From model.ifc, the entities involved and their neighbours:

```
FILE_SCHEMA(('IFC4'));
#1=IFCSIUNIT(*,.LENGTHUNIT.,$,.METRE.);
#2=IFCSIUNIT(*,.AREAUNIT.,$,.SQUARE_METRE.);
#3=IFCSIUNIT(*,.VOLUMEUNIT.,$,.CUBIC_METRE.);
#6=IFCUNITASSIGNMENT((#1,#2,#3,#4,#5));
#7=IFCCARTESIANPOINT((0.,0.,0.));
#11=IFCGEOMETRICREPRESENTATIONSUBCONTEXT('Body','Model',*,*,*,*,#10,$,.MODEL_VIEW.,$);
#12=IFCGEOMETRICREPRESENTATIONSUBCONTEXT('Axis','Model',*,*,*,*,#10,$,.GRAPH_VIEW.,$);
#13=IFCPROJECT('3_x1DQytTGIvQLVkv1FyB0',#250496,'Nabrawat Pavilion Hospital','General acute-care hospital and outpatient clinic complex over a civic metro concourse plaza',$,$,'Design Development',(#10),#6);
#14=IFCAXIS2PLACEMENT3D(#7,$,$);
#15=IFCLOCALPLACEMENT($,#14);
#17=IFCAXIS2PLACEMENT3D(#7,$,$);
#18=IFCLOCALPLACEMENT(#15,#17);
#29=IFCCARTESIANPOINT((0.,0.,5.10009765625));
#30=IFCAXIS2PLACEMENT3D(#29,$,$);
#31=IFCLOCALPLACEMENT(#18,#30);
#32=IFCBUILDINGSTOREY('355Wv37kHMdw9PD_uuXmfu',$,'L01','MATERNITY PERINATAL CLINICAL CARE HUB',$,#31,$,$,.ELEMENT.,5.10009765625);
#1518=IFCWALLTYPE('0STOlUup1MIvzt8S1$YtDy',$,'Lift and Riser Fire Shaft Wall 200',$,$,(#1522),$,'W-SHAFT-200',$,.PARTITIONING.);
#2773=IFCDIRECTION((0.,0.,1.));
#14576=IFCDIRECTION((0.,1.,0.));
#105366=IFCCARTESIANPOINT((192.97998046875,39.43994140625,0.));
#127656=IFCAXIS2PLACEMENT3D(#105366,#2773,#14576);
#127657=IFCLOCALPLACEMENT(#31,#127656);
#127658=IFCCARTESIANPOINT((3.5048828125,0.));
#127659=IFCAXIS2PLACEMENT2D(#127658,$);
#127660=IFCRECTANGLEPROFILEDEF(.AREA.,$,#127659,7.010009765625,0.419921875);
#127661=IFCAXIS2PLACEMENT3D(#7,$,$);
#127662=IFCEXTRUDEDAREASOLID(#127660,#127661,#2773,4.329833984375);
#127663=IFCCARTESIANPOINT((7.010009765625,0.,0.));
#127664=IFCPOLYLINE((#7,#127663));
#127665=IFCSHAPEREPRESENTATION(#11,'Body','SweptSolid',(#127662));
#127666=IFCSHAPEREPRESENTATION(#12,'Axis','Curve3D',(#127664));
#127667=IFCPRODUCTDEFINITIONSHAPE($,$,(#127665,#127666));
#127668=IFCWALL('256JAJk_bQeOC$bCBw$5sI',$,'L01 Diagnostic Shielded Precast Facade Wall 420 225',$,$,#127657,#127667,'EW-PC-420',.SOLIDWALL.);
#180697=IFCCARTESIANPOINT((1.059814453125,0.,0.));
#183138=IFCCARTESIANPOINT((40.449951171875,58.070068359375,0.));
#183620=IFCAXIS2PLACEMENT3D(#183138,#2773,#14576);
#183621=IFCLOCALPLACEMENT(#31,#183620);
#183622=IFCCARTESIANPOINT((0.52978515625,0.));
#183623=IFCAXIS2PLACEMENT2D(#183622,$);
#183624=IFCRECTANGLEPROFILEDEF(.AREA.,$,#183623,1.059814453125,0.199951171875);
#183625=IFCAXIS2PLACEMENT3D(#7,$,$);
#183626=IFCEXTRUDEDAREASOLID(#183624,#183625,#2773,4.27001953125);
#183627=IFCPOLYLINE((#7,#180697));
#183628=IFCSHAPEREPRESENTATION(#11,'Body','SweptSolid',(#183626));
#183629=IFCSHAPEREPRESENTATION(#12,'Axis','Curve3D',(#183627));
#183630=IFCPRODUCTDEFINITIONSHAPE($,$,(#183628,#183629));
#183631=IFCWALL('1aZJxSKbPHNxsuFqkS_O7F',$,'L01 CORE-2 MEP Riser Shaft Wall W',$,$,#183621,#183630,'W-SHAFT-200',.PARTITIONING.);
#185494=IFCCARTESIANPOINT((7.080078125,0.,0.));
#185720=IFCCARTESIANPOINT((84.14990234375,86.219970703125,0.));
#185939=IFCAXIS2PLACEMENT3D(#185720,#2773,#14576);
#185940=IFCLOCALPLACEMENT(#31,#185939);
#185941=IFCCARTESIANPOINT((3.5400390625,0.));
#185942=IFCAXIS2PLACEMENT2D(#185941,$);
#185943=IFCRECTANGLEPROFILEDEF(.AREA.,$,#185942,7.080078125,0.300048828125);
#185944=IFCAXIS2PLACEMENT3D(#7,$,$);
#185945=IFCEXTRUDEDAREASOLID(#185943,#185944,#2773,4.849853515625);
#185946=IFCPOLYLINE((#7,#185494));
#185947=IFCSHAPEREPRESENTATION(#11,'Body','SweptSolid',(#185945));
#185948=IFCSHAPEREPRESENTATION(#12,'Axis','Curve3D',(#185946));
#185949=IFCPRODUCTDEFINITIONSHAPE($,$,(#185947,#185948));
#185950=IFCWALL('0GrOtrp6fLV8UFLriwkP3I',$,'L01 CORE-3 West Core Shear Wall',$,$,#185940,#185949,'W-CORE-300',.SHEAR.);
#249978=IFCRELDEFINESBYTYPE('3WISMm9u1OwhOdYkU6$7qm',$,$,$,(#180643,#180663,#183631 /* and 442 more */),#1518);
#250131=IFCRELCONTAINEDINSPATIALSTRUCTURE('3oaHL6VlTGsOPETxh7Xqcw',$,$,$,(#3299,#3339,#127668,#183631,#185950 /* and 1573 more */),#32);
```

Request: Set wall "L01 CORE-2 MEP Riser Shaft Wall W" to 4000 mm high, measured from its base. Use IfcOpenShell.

```python
import ifcopenshell
import ifcopenshell.geom
import ifcopenshell.util.representation
import ifcopenshell.util.shape
import ifcopenshell.util.unit

model = ifcopenshell.open("model.ifc")
unit_scale = ifcopenshell.util.unit.calculate_unit_scale(model)
settings = ifcopenshell.geom.settings()


def volume(element):
    """Net volume in cubic metres, openings subtracted."""
    shape = ifcopenshell.geom.create_shape(settings, element)
    return ifcopenshell.util.shape.get_volume(shape.geometry)


wall = model.by_guid("1aZJxSKbPHNxsuFqkS_O7F")
before = volume(wall)

body = ifcopenshell.util.representation.get_representation(wall, "Model", "Body")
solid = body.Items[0]
old_height = solid.Depth
solid.Depth = 4 / unit_scale
after = volume(wall)

print(f"height {old_height:g} -> {solid.Depth:g}, volume {before:.3f} -> {after:.3f} m3")

model.write("model_rev.ifc")
```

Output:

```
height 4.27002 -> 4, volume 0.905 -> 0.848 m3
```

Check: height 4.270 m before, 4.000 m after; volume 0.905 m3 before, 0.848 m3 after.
